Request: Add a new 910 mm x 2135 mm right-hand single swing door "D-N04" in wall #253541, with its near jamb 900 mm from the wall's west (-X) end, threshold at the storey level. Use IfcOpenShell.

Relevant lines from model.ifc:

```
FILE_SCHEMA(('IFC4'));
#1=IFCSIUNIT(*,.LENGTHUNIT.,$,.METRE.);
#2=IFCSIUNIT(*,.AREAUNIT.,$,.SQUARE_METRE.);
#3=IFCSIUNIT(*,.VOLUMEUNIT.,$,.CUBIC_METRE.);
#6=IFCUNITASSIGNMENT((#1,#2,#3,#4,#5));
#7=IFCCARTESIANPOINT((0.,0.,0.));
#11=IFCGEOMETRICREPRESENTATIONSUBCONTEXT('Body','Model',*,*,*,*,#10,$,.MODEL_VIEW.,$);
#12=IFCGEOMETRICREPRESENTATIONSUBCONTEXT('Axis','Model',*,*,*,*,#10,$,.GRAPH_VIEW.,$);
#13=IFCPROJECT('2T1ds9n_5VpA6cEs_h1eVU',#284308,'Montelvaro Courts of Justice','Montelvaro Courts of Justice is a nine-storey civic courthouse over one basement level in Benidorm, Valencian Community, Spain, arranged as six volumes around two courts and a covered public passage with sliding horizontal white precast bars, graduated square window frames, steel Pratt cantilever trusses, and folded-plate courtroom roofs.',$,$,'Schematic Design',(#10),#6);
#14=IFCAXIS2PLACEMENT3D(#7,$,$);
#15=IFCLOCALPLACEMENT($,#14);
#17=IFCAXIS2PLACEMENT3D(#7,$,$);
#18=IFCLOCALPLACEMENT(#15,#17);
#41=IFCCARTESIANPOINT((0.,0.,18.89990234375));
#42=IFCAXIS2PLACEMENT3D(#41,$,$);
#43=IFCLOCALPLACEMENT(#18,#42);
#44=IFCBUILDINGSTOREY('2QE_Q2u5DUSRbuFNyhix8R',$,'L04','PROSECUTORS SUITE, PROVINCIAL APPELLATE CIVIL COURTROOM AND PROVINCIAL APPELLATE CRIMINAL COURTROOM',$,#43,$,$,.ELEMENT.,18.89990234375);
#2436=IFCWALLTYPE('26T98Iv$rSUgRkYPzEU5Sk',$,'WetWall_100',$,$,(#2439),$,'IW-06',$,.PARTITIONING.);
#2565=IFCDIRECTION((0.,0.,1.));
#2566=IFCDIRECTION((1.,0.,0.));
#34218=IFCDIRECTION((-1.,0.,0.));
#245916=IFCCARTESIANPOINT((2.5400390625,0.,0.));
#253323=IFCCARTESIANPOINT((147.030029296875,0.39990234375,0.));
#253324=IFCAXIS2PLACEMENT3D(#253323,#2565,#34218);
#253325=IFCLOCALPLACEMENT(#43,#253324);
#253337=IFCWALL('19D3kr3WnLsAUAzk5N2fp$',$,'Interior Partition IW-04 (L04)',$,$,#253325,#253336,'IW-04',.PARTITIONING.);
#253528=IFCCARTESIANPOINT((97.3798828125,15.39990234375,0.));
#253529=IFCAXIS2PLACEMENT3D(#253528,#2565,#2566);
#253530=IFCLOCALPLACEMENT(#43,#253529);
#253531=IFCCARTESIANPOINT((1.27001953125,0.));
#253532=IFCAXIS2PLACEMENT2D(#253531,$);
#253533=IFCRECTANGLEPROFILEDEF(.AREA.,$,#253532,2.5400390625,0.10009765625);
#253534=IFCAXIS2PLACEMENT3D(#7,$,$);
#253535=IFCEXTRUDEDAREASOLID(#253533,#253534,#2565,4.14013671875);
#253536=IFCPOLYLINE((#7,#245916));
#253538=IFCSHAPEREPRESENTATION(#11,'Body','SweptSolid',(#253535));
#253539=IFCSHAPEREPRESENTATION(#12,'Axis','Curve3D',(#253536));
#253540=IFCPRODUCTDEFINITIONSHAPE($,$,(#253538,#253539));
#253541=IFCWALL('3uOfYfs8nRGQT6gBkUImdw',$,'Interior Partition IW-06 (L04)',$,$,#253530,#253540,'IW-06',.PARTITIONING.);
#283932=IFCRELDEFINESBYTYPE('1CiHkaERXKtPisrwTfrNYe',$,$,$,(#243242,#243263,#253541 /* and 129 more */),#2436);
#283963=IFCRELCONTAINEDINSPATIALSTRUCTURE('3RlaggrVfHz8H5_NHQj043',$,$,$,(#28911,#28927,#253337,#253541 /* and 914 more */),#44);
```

```python
import numpy as np
import ifcopenshell
import ifcopenshell.api.feature
import ifcopenshell.api.geometry
import ifcopenshell.api.root
import ifcopenshell.api.spatial
import ifcopenshell.geom
import ifcopenshell.util.element
import ifcopenshell.util.placement
import ifcopenshell.util.representation
import ifcopenshell.util.shape
import ifcopenshell.util.unit

model = ifcopenshell.open("model.ifc")
unit_scale = ifcopenshell.util.unit.calculate_unit_scale(model)
settings = ifcopenshell.geom.settings()


def volume(element):
    """Net volume in cubic metres, openings subtracted."""
    shape = ifcopenshell.geom.create_shape(settings, element)
    return ifcopenshell.util.shape.get_volume(shape.geometry)


wall = model.by_guid("3uOfYfs8nRGQT6gBkUImdw")
storey = ifcopenshell.util.element.get_container(wall, ifc_class="IfcBuildingStorey")
context = ifcopenshell.util.representation.get_context(model, "Model", "Body", "MODEL_VIEW")
before = volume(wall)

width, height, from_end, sill = 0.91, 2.135, 0.9, 0.0  # metres

# The wall runs along its own X axis, and the end named is its -X end.
wall_shape = ifcopenshell.geom.create_shape(settings, wall)
x, y, z = ifcopenshell.util.shape.get_vertices(wall_shape.geometry).T
start = x.min() + from_end
face, thickness = float(y.min()), float(y.max() - y.min())
wall_matrix = ifcopenshell.util.placement.get_local_placement(wall.ObjectPlacement)
level = ifcopenshell.util.placement.get_local_placement(storey.ObjectPlacement)[2, 3]


def in_wall(x, y):
    """Placement at x, y metres in the wall's axes, at sill height."""
    matrix = wall_matrix.copy()
    matrix[:, 3] = wall_matrix @ np.array([x / unit_scale, y / unit_scale, 0.0, 1.0])
    matrix[2, 3] = level + sill / unit_scale
    return matrix


# Opening: a box that overshoots both wall faces by 50 mm.
opening = ifcopenshell.api.root.create_entity(model, ifc_class="IfcOpeningElement", predefined_type="OPENING")
box = ifcopenshell.api.geometry.add_wall_representation(
    model, context=context, length=width, height=height, thickness=thickness + 0.1
)
ifcopenshell.api.geometry.assign_representation(model, product=opening, representation=box)
ifcopenshell.api.geometry.edit_object_placement(model, product=opening, matrix=in_wall(start, face - 0.05), is_si=False)
ifcopenshell.api.feature.add_feature(model, feature=opening, element=wall)

door = ifcopenshell.api.root.create_entity(model, ifc_class="IfcDoor", name="D-N04", predefined_type="DOOR")
door.OverallWidth, door.OverallHeight = width / unit_scale, height / unit_scale
door.OperationType = "SINGLE_SWING_RIGHT"
body = ifcopenshell.api.geometry.add_door_representation(
    model,
    context=context,
    overall_width=door.OverallWidth,
    overall_height=door.OverallHeight,
    operation_type="SINGLE_SWING_RIGHT",
    lining_properties={"LiningDepth": thickness / unit_scale, "ThresholdDepth": thickness / unit_scale},
)
ifcopenshell.api.geometry.assign_representation(model, product=door, representation=body)
ifcopenshell.api.spatial.assign_container(model, products=[door], relating_structure=storey)
ifcopenshell.api.feature.add_filling(model, opening=opening, element=door)

# The lining spans the wall, so the door starts at the wall face.
ifcopenshell.api.geometry.edit_object_placement(model, product=door, matrix=in_wall(start, face), is_si=False)

after = volume(wall)

print(f"wall volume {before:.3f} -> {after:.3f} m3")

model.write("model_rev.ifc")
```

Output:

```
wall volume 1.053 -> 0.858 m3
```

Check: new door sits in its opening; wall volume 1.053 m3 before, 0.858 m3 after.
